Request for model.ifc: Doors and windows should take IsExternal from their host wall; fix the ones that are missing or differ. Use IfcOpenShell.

First a look at what the model holds.

```python
import ifcopenshell
import ifcopenshell.util.element

model = ifcopenshell.open("model.ifc")
print(model.schema)
seen = {}
for e in model.by_type("IfcDoor") + model.by_type("IfcWindow"):
    if not e.FillsVoids:
        continue
    host = e.FillsVoids[0].RelatingOpeningElement.VoidsElements[0].RelatingBuildingElement
    own = ifcopenshell.util.element.get_pset(e, f"Pset_{e.is_a()[3:].removesuffix('StandardCase')}Common", "IsExternal")
    wall = ifcopenshell.util.element.get_pset(host, "Pset_WallCommon", "IsExternal")
    seen[e.is_a(), own, wall] = seen.get((e.is_a(), own, wall), 0) + 1
for (cls, own, wall), count in sorted(seen.items(), key=str):
    print(count, cls, "IsExternal:", own, "| host wall:", wall)
```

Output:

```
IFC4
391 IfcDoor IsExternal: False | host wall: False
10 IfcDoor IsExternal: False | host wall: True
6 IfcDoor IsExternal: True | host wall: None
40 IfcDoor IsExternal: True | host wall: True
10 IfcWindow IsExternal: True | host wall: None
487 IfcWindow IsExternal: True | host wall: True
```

```python
import ifcopenshell
import ifcopenshell.api.pset
import ifcopenshell.util.element

model = ifcopenshell.open("model.ifc")

count = 0
for ifc_class, pset_name in (("IfcDoor", "Pset_DoorCommon"), ("IfcWindow", "Pset_WindowCommon")):
    for e in model.by_type(ifc_class):
        if not e.FillsVoids:
            continue
        host = e.FillsVoids[0].RelatingOpeningElement.VoidsElements[0].RelatingBuildingElement
        external = ifcopenshell.util.element.get_pset(host, "Pset_WallCommon", "IsExternal")
        if external is None or ifcopenshell.util.element.get_pset(e, pset_name, "IsExternal") == external:
            continue
        pset = ifcopenshell.api.pset.add_pset(model, product=e, name=pset_name)
        ifcopenshell.api.pset.edit_pset(model, pset=pset, properties={"IsExternal": external})
        count += 1

print(count, "updated")

model.write("model_v2.ifc")
```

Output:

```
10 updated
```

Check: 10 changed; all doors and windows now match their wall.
